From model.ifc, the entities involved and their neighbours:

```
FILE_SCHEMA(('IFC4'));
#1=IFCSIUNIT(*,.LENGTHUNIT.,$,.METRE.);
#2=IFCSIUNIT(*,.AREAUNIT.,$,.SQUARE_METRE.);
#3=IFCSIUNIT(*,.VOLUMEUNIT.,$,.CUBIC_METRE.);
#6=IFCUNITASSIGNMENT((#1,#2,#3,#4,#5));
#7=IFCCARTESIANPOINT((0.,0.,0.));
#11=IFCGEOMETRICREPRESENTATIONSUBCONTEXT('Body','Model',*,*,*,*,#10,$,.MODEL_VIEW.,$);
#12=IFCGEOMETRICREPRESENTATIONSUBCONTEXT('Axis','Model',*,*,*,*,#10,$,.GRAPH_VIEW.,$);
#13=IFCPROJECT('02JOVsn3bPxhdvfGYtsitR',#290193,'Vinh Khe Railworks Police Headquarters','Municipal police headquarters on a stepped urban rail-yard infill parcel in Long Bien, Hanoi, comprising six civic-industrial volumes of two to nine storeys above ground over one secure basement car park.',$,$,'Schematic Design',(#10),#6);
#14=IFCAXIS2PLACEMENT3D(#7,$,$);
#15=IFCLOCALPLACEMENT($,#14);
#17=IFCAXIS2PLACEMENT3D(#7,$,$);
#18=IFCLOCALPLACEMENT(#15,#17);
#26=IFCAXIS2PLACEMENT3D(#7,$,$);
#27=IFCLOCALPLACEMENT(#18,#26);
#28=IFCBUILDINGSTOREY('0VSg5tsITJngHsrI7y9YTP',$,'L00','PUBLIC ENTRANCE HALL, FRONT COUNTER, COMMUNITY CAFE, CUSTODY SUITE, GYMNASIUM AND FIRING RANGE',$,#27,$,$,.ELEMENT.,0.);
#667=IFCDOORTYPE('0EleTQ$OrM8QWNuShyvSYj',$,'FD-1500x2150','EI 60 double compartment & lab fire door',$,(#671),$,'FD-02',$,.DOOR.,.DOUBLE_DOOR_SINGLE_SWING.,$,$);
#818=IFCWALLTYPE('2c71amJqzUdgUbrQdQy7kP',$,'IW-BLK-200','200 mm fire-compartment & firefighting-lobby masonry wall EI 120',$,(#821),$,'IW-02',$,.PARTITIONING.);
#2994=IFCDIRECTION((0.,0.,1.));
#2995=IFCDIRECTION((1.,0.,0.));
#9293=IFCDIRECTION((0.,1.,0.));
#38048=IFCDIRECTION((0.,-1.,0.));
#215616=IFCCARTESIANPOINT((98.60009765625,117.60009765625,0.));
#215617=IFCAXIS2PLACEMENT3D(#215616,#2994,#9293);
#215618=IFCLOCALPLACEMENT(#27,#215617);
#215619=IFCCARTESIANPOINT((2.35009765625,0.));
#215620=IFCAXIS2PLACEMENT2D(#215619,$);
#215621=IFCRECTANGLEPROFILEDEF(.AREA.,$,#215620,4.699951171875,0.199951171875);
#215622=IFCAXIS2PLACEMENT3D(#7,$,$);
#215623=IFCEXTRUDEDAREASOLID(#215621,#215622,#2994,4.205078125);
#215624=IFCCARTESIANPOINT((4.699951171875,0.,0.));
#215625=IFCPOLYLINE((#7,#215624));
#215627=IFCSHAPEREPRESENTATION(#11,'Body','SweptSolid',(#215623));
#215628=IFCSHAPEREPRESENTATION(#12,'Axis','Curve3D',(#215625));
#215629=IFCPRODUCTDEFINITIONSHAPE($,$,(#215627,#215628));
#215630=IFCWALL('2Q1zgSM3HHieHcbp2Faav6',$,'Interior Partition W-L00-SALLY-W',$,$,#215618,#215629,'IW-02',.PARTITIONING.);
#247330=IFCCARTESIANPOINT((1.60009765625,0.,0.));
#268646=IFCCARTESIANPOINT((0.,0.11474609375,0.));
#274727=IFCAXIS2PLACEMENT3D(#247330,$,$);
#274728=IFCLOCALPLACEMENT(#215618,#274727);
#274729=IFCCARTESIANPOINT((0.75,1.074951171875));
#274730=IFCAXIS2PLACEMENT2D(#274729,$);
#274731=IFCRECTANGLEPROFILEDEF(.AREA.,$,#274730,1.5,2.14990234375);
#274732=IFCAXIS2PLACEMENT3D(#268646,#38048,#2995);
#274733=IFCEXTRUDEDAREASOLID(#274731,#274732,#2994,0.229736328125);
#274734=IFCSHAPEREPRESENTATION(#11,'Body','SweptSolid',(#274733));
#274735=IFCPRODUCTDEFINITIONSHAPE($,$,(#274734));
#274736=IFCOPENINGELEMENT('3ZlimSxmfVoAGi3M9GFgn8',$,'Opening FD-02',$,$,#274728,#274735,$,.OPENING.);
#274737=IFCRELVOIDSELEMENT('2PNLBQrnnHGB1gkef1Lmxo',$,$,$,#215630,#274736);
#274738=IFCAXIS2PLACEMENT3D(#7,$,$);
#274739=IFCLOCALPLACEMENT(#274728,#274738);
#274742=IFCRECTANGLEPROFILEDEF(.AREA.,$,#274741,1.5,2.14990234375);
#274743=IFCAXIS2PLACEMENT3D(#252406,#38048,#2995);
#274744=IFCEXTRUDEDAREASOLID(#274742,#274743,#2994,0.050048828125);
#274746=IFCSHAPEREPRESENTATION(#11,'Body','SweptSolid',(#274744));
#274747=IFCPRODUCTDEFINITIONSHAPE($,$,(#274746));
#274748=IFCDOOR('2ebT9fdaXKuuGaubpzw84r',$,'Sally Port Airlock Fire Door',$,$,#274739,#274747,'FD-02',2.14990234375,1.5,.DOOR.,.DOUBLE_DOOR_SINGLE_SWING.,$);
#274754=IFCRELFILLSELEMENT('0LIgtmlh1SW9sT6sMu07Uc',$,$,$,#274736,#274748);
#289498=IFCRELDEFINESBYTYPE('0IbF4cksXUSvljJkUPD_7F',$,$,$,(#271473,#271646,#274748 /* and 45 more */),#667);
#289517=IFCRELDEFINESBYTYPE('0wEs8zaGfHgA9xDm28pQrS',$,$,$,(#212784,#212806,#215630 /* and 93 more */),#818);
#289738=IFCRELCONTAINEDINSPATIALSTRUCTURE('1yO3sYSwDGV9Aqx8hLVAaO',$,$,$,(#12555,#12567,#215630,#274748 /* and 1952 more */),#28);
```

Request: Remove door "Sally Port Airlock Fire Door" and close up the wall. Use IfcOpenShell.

```python
import ifcopenshell
import ifcopenshell.api.feature
import ifcopenshell.api.root
import ifcopenshell.geom
import ifcopenshell.util.shape

model = ifcopenshell.open("model.ifc")
settings = ifcopenshell.geom.settings()


def volume(element):
    """Net volume in cubic metres, openings subtracted."""
    shape = ifcopenshell.geom.create_shape(settings, element)
    return ifcopenshell.util.shape.get_volume(shape.geometry)


door = model.by_id(274748)
opening = door.FillsVoids[0].RelatingOpeningElement
wall = opening.VoidsElements[0].RelatingBuildingElement
before = volume(wall)

ifcopenshell.api.root.remove_product(model, product=door)
ifcopenshell.api.feature.remove_feature(model, feature=opening)

after = volume(wall)

print(f"wall volume {before:.3f} -> {after:.3f} m3")

model.write("model_v2.ifc")
```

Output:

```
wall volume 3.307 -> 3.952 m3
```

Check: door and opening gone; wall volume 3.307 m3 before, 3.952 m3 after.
